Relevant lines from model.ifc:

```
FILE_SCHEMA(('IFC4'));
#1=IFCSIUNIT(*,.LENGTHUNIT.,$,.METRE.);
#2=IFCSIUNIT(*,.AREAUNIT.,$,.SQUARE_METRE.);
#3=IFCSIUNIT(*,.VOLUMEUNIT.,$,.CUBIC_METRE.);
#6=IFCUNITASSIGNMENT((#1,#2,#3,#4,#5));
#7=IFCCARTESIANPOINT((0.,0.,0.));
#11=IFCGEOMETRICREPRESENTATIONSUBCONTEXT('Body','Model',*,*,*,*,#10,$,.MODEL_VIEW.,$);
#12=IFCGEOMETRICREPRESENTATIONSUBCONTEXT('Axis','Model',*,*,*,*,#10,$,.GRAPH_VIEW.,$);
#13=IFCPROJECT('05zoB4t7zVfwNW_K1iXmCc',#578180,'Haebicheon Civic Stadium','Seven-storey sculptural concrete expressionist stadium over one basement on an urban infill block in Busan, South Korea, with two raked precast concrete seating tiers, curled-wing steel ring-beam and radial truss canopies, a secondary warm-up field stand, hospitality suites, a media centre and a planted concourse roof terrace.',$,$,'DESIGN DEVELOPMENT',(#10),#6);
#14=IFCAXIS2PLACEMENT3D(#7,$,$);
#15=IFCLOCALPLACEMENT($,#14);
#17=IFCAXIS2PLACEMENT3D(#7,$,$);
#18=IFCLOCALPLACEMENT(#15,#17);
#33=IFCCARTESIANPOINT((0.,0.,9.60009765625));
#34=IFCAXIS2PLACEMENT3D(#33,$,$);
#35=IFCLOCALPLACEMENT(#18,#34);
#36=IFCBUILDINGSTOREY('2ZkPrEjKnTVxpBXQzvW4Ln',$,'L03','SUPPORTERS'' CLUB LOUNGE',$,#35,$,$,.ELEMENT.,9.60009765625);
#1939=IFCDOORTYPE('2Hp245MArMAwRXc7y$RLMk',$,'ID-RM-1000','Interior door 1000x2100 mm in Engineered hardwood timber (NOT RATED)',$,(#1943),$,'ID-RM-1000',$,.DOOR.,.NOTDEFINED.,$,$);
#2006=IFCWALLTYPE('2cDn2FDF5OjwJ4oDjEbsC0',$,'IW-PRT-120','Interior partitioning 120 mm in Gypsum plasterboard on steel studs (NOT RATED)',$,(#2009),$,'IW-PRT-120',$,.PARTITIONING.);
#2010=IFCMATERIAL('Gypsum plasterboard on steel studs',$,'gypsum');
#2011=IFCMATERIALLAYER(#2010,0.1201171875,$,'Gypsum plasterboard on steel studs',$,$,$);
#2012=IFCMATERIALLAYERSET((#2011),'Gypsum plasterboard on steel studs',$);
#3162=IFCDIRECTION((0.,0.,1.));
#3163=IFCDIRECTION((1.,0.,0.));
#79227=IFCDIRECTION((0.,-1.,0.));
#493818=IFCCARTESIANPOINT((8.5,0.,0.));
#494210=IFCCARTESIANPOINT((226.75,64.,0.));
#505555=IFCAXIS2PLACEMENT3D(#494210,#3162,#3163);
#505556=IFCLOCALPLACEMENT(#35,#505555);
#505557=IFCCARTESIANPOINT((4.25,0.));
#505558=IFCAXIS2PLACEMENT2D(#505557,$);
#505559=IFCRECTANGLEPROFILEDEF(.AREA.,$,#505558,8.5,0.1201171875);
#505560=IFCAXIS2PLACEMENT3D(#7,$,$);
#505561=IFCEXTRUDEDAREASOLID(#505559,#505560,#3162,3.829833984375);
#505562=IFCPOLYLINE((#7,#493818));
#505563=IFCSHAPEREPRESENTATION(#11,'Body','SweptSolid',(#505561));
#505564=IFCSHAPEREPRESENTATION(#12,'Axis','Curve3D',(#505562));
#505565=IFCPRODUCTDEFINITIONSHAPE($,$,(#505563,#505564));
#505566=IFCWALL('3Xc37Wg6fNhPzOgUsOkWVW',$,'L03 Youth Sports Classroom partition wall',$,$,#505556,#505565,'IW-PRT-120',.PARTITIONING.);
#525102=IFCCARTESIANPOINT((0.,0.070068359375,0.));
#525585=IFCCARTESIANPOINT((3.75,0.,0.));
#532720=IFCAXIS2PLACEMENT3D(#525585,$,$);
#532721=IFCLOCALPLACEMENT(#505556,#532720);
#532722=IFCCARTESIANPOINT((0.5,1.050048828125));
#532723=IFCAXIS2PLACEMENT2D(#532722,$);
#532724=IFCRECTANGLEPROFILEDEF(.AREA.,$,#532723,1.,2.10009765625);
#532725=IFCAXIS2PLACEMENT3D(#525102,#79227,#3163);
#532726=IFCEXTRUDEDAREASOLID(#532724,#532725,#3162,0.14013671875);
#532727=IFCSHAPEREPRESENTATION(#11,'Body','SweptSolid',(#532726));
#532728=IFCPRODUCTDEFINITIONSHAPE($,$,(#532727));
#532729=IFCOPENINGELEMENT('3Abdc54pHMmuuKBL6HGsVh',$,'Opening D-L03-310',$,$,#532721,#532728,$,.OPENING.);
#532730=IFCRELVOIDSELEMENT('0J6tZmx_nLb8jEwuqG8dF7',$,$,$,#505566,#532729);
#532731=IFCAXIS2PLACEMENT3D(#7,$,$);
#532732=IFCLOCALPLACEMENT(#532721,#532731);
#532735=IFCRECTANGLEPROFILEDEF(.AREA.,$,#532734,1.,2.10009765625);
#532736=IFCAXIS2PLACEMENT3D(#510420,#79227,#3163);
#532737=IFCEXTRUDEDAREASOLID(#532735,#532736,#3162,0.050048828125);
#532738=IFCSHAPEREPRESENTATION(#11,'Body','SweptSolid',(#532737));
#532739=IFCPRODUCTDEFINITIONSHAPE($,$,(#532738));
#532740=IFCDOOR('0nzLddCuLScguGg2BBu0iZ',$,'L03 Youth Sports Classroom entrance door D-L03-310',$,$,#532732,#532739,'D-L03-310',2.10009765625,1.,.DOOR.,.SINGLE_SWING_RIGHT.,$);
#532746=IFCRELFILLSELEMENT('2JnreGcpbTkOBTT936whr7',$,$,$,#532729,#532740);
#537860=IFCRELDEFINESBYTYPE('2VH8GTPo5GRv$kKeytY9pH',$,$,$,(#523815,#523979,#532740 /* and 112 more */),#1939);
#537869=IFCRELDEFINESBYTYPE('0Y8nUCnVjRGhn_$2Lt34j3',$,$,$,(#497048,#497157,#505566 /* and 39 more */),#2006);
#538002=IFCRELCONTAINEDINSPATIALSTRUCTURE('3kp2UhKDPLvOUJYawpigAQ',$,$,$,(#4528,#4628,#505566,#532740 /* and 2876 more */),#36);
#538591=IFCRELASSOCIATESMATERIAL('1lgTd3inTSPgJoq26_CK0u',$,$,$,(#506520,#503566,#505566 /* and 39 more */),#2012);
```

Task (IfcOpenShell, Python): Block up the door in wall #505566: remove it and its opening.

```python
import ifcopenshell
import ifcopenshell.api.feature
import ifcopenshell.api.root
import ifcopenshell.geom
import ifcopenshell.util.shape

model = ifcopenshell.open("model.ifc")
settings = ifcopenshell.geom.settings()


def volume(element):
    """Net volume in cubic metres, openings subtracted."""
    shape = ifcopenshell.geom.create_shape(settings, element)
    return ifcopenshell.util.shape.get_volume(shape.geometry)


door = model.by_guid("0nzLddCuLScguGg2BBu0iZ")
opening = door.FillsVoids[0].RelatingOpeningElement
wall = opening.VoidsElements[0].RelatingBuildingElement
before = volume(wall)

ifcopenshell.api.root.remove_product(model, product=door)
ifcopenshell.api.feature.remove_feature(model, feature=opening)

after = volume(wall)

print(f"wall volume {before:.3f} -> {after:.3f} m3")

model.write("model_edited.ifc")
```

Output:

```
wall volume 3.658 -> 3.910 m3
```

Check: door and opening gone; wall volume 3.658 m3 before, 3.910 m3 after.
